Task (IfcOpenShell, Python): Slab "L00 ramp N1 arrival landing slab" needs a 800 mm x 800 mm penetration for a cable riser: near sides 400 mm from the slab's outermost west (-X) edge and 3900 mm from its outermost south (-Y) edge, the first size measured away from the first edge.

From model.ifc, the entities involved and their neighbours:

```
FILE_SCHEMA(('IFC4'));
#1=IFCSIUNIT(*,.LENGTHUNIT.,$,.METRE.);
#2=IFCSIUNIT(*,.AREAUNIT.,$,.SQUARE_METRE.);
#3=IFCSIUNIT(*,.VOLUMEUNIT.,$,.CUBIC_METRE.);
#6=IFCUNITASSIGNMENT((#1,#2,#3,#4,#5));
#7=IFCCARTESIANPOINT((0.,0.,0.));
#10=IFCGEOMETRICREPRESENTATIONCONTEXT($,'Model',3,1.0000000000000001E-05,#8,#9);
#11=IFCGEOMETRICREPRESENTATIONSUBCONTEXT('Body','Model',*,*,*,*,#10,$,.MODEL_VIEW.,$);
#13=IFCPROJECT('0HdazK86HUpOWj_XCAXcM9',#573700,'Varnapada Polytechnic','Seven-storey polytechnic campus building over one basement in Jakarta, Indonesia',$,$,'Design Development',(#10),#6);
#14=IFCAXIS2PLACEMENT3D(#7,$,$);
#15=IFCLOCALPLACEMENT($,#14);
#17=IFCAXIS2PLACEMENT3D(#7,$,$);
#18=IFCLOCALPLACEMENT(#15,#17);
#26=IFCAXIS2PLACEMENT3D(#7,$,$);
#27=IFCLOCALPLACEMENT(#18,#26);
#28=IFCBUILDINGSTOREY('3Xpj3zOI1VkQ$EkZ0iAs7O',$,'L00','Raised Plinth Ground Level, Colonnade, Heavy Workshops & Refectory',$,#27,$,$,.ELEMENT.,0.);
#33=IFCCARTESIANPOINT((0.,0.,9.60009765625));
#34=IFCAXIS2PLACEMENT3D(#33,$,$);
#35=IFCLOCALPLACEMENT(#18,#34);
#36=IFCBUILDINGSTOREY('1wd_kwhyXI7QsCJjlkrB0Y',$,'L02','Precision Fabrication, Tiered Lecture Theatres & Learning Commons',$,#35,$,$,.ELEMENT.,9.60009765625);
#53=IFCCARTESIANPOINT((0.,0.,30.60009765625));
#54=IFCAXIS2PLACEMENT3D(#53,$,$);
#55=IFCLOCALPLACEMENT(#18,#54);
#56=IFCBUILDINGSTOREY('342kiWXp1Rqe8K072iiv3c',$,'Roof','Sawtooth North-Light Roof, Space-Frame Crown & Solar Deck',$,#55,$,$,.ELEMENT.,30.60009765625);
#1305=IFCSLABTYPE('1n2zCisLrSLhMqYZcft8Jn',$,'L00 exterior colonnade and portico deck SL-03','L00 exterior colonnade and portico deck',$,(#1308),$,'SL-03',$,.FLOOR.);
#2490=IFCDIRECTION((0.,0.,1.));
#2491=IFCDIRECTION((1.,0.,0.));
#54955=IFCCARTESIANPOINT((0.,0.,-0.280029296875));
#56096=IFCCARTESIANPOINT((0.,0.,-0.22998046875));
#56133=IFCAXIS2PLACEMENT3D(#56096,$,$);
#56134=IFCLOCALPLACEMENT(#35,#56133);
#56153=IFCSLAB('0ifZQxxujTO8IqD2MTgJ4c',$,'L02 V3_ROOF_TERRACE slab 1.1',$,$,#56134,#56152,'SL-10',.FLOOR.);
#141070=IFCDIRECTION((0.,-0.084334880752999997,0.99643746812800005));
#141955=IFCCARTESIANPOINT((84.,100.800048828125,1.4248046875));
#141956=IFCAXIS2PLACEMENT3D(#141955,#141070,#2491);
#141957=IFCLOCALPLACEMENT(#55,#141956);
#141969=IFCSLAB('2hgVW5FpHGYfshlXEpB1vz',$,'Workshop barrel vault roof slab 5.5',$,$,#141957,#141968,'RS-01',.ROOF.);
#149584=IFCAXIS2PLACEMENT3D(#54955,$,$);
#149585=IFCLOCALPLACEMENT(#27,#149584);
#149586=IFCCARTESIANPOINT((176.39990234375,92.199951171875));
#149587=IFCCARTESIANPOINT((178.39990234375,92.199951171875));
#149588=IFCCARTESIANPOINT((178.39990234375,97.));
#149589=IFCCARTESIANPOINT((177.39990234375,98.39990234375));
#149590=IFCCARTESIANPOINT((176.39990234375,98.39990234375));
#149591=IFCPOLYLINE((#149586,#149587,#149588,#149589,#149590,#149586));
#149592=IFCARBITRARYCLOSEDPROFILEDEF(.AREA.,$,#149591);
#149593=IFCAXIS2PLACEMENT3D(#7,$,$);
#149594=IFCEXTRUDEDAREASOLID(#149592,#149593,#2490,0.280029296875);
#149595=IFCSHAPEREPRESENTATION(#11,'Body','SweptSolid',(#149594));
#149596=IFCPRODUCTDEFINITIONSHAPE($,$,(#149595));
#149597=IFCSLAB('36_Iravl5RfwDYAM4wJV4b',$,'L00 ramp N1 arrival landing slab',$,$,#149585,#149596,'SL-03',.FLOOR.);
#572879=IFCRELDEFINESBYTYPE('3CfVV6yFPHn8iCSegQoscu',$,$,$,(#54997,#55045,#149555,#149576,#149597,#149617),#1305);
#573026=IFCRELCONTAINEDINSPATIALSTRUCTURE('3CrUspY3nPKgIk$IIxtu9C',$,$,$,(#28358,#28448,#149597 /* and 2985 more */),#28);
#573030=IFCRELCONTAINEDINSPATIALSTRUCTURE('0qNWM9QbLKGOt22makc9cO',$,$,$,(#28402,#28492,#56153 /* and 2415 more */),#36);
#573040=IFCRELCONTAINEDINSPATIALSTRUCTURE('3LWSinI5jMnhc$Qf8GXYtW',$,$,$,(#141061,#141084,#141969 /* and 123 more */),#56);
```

```python
import numpy as np
import ifcopenshell
import ifcopenshell.api.feature
import ifcopenshell.api.geometry
import ifcopenshell.api.root
import ifcopenshell.geom
import ifcopenshell.util.placement
import ifcopenshell.util.representation
import ifcopenshell.util.shape
import ifcopenshell.util.unit

model = ifcopenshell.open("model.ifc")
unit_scale = ifcopenshell.util.unit.calculate_unit_scale(model)
settings = ifcopenshell.geom.settings()


def volume(element):
    """Net volume in cubic metres, openings subtracted."""
    shape = ifcopenshell.geom.create_shape(settings, element)
    return ifcopenshell.util.shape.get_volume(shape.geometry)


slab = model.by_id(149597)
before = volume(slab)

# Extent in the slab's own axes, in metres. The edges named are its -X and -Y sides.
slab_shape = ifcopenshell.geom.create_shape(settings, slab)
vertices = ifcopenshell.util.shape.get_vertices(slab_shape.geometry)
x_min, y_min, bottom = vertices.min(axis=0)
top = vertices[:, 2].max()

opening = ifcopenshell.api.root.create_entity(model, ifc_class="IfcOpeningElement", name="Cable riser opening", predefined_type="OPENING")
context = ifcopenshell.util.representation.get_context(model, "Model", "Body", "MODEL_VIEW")
width, depth = 0.8, 0.8
outline = [(0.0, 0.0), (width, 0.0), (width, depth), (0.0, depth), (0.0, 0.0)]
# Overshoot both faces by 50 mm so the cut is clean.
shape = ifcopenshell.api.geometry.add_slab_representation(
    model, context=context, depth=top - bottom + 0.1, polyline=outline
)
ifcopenshell.api.geometry.assign_representation(model, product=opening, representation=shape)

matrix = ifcopenshell.util.placement.get_local_placement(slab.ObjectPlacement)
matrix[:, 3] = matrix @ np.append(np.array([x_min + 0.4, y_min + 3.9, bottom - 0.05]) / unit_scale, 1.0)
ifcopenshell.api.geometry.edit_object_placement(model, product=opening, matrix=matrix, is_si=False)
ifcopenshell.api.feature.add_feature(model, feature=opening, element=slab)

after = volume(slab)

print(f"slab volume {before:.3f} -> {after:.3f} m3")

model.write("model-out.ifc")
```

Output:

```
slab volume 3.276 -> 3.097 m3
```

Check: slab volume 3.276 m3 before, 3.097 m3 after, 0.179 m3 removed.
